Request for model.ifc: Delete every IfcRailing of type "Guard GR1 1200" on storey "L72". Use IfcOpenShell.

First a look at what the model holds.

```python
import ifcopenshell
import ifcopenshell.util.element

model = ifcopenshell.open("model.ifc")
print(model.schema)
storey = next(s for s in model.by_type("IfcBuildingStorey") if s.Name == "L72")
railings = [e for e in ifcopenshell.util.element.get_decomposition(storey) if e.is_a("IfcRailing")]
seen = {}
for e in railings:
    element_type = ifcopenshell.util.element.get_type(e)
    name = element_type.Name if element_type not in (None, e) else None
    seen[name] = seen.get(name, 0) + 1
for name, count in sorted(seen.items(), key=str):
    print(count, "x", name)
```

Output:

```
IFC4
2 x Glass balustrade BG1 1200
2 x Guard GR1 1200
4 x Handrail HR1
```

```python
import ifcopenshell
import ifcopenshell.api.root
import ifcopenshell.util.element

model = ifcopenshell.open("model.ifc")

storey = next(s for s in model.by_type("IfcBuildingStorey") if s.Name == "L72")
railings = [e for e in ifcopenshell.util.element.get_decomposition(storey) if e.is_a("IfcRailing")]
targets = [e for e in railings if (t := ifcopenshell.util.element.get_type(e)) not in (None, e) and t.Name == "Guard GR1 1200"]

for e in targets:
    ifcopenshell.api.root.remove_product(model, product=e)
print(len(targets), "removed")

model.write("model_v2.ifc")
```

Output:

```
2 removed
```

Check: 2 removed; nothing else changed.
